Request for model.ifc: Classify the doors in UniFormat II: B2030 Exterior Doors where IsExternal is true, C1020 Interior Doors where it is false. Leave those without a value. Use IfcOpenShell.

First a look at what the model holds.

```python
import ifcopenshell
import ifcopenshell.util.element

model = ifcopenshell.open("model.ifc")
print(model.schema)
print("classifications:", [c.Name for c in model.by_type("IfcClassification")])
values = [ifcopenshell.util.element.get_pset(e, "Pset_DoorCommon", "IsExternal") for e in model.by_type("IfcDoor")]
for value in (True, False, None):
    print("IsExternal", value, values.count(value))
```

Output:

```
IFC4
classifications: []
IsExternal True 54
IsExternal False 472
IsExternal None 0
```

```python
import ifcopenshell
import ifcopenshell.api.classification
import ifcopenshell.util.element

model = ifcopenshell.open("model.ifc")

system = ifcopenshell.api.classification.add_classification(model, classification="UniFormat II")

doors = model.by_type("IfcDoor")
external = {e: ifcopenshell.util.element.get_pset(e, "Pset_DoorCommon", "IsExternal") for e in doors}
for flag, code, name in ((True, "B2030", "Exterior Doors"), (False, "C1020", "Interior Doors")):
    products = [e for e in doors if external[e] is flag]
    ifcopenshell.api.classification.add_reference(
        model, products=products, classification=system, identification=code, name=name
    )
    print(code, len(products))

model.write("model_edited.ifc")
```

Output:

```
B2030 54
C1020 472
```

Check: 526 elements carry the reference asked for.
